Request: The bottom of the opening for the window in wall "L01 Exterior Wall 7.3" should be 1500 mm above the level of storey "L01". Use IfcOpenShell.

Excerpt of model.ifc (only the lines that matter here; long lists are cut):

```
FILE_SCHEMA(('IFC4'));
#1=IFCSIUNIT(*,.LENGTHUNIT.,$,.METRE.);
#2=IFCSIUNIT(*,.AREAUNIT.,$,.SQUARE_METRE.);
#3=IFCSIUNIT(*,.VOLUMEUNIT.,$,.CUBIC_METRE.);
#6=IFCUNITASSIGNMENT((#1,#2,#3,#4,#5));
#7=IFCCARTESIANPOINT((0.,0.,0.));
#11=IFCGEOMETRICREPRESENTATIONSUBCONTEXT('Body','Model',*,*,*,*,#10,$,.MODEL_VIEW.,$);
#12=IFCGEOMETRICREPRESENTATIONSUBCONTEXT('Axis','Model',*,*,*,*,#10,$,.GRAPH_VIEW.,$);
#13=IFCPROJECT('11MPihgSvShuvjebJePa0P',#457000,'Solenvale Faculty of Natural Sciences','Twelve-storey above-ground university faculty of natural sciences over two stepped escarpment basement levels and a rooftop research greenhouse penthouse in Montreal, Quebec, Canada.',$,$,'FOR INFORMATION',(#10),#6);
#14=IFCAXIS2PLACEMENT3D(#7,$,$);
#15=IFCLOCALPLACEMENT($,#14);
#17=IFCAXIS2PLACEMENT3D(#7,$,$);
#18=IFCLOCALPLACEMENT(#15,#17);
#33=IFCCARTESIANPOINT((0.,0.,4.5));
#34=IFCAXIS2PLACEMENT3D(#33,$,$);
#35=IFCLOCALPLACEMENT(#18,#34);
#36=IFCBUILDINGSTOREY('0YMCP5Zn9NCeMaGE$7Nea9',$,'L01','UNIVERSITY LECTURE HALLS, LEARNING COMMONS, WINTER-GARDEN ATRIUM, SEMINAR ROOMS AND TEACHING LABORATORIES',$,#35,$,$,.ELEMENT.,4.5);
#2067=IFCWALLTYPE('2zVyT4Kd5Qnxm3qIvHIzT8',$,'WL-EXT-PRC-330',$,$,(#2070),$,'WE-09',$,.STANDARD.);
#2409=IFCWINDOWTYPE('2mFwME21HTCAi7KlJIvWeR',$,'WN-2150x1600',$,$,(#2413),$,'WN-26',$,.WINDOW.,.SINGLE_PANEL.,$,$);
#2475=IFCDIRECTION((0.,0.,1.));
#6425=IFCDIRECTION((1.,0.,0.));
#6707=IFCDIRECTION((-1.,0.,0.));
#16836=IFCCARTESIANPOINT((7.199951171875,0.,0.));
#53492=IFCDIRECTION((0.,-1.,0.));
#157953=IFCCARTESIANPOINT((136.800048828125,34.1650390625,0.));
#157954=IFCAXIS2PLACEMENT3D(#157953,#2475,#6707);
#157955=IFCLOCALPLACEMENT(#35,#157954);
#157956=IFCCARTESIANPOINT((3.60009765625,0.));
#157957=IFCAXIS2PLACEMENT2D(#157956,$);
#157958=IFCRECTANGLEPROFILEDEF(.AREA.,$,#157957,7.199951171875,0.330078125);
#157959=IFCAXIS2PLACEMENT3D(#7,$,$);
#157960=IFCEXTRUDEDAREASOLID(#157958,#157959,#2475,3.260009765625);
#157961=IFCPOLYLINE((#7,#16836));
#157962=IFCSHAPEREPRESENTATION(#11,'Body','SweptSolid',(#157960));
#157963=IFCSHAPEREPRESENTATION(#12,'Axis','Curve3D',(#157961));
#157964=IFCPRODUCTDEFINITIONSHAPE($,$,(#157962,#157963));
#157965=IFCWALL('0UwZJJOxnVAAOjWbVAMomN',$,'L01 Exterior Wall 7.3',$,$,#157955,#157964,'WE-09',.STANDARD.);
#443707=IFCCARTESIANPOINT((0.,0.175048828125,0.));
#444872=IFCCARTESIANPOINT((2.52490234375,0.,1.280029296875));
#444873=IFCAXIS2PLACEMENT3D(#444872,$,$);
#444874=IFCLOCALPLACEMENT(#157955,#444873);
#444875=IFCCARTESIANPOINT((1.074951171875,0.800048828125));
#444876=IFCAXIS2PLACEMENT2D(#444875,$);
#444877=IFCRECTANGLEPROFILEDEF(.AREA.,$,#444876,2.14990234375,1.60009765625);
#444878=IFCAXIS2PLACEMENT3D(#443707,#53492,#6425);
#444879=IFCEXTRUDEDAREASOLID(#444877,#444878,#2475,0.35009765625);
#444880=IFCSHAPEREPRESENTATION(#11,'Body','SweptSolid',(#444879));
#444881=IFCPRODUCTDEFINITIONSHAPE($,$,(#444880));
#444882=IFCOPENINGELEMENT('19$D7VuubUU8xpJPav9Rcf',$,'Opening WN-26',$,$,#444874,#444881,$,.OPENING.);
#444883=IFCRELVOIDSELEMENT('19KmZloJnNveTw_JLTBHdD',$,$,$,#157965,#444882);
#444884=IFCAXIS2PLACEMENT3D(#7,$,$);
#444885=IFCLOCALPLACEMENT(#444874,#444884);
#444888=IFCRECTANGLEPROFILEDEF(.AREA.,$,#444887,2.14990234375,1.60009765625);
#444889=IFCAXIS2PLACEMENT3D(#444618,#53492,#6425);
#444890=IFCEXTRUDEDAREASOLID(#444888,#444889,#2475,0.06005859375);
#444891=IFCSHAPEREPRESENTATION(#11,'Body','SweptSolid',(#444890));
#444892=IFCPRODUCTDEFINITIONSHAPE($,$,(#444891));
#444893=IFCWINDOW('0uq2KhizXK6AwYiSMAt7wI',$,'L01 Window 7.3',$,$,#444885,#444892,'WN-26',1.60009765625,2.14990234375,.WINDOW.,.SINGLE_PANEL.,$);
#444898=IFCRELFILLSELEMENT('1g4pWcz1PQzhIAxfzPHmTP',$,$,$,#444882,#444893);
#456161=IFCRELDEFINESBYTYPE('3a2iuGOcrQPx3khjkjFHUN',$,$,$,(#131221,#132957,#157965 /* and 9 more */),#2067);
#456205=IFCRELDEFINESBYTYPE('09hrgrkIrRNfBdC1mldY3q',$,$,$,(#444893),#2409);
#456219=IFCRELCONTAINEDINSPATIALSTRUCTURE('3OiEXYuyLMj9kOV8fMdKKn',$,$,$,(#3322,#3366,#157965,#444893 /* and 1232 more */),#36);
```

```python
import numpy as np
import ifcopenshell
import ifcopenshell.api.geometry
import ifcopenshell.geom
import ifcopenshell.util.element
import ifcopenshell.util.placement
import ifcopenshell.util.shape
import ifcopenshell.util.unit

model = ifcopenshell.open("model.ifc")
unit_scale = ifcopenshell.util.unit.calculate_unit_scale(model)

window = model.by_guid("0uq2KhizXK6AwYiSMAt7wI")
opening = window.FillsVoids[0].RelatingOpeningElement
storey = ifcopenshell.util.element.get_container(window, ifc_class="IfcBuildingStorey")
level = ifcopenshell.util.placement.get_local_placement(storey.ObjectPlacement)[2, 3]

# The opening's origin need not be at the sill, so measure its lowest point.
shape = ifcopenshell.geom.create_shape(ifcopenshell.geom.settings(), opening)
bottom = ifcopenshell.util.shape.get_shape_bottom_elevation(shape, shape.geometry) / unit_scale
dz = level + 1.5 / unit_scale - bottom

shift = np.array([0.0, 0.0, dz])
# The window is placed relative to its opening, so it follows when the opening moves.
matrix = ifcopenshell.util.placement.get_local_placement(opening.ObjectPlacement)
matrix[:3, 3] += shift
ifcopenshell.api.geometry.edit_object_placement(
    model, product=opening, matrix=matrix, is_si=False, should_transform_children=True
)

print(f"moved by {dz * unit_scale:+.3f} m")

model.write("model-out.ifc")
```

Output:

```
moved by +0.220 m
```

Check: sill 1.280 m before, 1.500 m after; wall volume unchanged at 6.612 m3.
